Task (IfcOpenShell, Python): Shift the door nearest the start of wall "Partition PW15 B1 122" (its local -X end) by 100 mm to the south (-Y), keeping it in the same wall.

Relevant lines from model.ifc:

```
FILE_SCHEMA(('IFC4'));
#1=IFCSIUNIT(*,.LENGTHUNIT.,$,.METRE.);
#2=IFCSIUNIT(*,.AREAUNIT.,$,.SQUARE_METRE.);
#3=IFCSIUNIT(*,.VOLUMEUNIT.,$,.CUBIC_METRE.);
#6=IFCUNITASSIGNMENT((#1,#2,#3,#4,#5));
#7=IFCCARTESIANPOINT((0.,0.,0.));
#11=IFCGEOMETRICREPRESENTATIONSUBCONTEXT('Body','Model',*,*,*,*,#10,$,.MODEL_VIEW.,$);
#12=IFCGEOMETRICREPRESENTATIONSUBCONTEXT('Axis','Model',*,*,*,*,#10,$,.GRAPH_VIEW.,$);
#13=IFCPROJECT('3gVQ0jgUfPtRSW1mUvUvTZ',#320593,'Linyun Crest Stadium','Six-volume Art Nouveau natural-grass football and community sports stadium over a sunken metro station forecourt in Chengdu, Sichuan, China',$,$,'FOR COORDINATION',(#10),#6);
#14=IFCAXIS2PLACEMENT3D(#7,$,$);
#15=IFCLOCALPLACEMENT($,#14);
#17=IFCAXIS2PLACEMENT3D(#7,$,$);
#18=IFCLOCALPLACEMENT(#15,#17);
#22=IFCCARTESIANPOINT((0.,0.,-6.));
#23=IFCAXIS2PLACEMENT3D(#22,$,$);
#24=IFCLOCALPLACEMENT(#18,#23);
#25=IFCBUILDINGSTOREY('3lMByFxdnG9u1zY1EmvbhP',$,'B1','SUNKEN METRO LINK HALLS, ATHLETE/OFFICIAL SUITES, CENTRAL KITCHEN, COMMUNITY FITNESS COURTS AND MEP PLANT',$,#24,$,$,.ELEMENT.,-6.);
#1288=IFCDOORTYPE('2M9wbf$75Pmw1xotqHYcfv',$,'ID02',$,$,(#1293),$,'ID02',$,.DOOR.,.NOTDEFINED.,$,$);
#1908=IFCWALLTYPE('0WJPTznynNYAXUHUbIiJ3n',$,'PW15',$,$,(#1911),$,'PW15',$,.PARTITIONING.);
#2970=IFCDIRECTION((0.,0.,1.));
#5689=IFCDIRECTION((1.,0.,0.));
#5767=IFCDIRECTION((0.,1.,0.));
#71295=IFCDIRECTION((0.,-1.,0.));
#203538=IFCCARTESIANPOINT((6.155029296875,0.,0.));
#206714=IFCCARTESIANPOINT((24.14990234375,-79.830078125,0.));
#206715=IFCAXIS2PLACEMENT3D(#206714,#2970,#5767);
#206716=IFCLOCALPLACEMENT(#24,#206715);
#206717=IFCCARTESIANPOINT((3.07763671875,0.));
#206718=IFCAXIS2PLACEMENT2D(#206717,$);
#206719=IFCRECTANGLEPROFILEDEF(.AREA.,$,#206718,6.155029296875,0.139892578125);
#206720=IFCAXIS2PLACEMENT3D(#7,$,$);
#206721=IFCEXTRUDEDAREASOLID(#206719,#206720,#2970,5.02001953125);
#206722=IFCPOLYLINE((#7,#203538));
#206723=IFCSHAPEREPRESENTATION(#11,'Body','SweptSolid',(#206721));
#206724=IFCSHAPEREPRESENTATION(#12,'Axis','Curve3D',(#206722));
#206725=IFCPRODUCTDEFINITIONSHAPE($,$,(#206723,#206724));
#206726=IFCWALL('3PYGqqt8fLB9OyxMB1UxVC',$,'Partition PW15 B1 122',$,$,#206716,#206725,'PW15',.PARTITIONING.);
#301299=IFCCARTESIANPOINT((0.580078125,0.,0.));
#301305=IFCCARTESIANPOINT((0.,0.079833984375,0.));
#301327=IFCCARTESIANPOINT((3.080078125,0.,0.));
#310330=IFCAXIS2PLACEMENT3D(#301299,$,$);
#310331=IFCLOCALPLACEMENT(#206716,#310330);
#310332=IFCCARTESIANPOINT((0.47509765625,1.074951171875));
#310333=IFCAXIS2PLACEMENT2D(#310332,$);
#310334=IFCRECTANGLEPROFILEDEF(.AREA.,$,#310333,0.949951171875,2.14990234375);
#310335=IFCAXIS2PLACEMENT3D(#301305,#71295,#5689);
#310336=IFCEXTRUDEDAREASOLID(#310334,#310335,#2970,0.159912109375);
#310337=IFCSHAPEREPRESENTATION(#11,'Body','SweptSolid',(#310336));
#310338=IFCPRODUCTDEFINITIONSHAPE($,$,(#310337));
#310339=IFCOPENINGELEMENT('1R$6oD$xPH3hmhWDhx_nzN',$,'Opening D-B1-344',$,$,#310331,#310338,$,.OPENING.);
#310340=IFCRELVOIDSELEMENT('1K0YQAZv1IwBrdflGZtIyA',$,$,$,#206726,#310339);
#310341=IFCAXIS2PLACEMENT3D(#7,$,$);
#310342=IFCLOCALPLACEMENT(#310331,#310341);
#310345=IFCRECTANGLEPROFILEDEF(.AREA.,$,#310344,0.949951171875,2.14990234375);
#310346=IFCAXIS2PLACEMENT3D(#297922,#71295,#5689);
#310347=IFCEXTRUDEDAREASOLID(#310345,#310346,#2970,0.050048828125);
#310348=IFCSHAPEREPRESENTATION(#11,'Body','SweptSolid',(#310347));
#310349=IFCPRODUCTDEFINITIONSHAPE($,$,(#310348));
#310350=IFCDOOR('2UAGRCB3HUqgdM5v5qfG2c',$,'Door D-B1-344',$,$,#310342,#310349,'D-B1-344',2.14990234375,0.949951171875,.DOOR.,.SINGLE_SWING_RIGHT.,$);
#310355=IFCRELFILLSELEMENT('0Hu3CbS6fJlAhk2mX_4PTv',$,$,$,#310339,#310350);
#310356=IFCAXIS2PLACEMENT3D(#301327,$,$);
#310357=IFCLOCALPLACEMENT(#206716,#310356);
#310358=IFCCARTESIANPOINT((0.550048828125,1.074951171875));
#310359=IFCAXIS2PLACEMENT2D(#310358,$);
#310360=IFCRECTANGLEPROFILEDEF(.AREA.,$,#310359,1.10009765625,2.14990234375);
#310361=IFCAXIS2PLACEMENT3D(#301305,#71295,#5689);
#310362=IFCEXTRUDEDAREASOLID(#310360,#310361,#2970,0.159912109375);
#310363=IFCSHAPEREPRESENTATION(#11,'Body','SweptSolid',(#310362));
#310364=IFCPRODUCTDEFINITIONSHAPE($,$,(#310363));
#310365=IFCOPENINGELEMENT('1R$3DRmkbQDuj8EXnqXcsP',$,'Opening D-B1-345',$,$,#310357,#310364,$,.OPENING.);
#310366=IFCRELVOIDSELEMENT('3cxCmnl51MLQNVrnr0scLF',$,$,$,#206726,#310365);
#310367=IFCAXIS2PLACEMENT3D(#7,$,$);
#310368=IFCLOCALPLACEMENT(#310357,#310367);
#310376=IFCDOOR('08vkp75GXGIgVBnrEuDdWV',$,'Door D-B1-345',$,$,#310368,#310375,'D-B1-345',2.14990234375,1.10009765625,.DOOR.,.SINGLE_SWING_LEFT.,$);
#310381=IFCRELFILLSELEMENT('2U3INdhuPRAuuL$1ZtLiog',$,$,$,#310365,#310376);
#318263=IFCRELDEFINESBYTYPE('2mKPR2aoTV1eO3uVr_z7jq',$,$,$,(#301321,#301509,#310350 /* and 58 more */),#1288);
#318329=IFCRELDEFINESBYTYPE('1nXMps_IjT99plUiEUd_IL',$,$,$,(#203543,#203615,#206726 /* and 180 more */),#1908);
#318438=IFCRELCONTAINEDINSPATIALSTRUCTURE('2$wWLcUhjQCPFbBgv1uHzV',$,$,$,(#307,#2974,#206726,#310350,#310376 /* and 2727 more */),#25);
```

```python
import ifcopenshell
import ifcopenshell.api.geometry
import ifcopenshell.util.placement
import ifcopenshell.util.unit

model = ifcopenshell.open("model.ifc")
unit_scale = ifcopenshell.util.unit.calculate_unit_scale(model)

door = model.by_guid("2UAGRCB3HUqgdM5v5qfG2c")
opening = door.FillsVoids[0].RelatingOpeningElement
wall = opening.VoidsElements[0].RelatingBuildingElement

wall_matrix = ifcopenshell.util.placement.get_local_placement(wall.ObjectPlacement)
shift = wall_matrix[:3, 0] * -0.1 / unit_scale
before = ifcopenshell.util.placement.get_local_placement(door.ObjectPlacement)[:3, 3].copy()

# The door is placed relative to its opening, so it follows when the opening moves.
matrix = ifcopenshell.util.placement.get_local_placement(opening.ObjectPlacement)
matrix[:3, 3] += shift
ifcopenshell.api.geometry.edit_object_placement(
    model, product=opening, matrix=matrix, is_si=False, should_transform_children=True
)

after = ifcopenshell.util.placement.get_local_placement(door.ObjectPlacement)[:3, 3]
print("door moved by", (after - before).round(3) + 0.0)

model.write("model_rev.ifc")
```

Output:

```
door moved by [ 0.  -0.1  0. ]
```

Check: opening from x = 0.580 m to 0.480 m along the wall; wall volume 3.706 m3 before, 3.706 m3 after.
